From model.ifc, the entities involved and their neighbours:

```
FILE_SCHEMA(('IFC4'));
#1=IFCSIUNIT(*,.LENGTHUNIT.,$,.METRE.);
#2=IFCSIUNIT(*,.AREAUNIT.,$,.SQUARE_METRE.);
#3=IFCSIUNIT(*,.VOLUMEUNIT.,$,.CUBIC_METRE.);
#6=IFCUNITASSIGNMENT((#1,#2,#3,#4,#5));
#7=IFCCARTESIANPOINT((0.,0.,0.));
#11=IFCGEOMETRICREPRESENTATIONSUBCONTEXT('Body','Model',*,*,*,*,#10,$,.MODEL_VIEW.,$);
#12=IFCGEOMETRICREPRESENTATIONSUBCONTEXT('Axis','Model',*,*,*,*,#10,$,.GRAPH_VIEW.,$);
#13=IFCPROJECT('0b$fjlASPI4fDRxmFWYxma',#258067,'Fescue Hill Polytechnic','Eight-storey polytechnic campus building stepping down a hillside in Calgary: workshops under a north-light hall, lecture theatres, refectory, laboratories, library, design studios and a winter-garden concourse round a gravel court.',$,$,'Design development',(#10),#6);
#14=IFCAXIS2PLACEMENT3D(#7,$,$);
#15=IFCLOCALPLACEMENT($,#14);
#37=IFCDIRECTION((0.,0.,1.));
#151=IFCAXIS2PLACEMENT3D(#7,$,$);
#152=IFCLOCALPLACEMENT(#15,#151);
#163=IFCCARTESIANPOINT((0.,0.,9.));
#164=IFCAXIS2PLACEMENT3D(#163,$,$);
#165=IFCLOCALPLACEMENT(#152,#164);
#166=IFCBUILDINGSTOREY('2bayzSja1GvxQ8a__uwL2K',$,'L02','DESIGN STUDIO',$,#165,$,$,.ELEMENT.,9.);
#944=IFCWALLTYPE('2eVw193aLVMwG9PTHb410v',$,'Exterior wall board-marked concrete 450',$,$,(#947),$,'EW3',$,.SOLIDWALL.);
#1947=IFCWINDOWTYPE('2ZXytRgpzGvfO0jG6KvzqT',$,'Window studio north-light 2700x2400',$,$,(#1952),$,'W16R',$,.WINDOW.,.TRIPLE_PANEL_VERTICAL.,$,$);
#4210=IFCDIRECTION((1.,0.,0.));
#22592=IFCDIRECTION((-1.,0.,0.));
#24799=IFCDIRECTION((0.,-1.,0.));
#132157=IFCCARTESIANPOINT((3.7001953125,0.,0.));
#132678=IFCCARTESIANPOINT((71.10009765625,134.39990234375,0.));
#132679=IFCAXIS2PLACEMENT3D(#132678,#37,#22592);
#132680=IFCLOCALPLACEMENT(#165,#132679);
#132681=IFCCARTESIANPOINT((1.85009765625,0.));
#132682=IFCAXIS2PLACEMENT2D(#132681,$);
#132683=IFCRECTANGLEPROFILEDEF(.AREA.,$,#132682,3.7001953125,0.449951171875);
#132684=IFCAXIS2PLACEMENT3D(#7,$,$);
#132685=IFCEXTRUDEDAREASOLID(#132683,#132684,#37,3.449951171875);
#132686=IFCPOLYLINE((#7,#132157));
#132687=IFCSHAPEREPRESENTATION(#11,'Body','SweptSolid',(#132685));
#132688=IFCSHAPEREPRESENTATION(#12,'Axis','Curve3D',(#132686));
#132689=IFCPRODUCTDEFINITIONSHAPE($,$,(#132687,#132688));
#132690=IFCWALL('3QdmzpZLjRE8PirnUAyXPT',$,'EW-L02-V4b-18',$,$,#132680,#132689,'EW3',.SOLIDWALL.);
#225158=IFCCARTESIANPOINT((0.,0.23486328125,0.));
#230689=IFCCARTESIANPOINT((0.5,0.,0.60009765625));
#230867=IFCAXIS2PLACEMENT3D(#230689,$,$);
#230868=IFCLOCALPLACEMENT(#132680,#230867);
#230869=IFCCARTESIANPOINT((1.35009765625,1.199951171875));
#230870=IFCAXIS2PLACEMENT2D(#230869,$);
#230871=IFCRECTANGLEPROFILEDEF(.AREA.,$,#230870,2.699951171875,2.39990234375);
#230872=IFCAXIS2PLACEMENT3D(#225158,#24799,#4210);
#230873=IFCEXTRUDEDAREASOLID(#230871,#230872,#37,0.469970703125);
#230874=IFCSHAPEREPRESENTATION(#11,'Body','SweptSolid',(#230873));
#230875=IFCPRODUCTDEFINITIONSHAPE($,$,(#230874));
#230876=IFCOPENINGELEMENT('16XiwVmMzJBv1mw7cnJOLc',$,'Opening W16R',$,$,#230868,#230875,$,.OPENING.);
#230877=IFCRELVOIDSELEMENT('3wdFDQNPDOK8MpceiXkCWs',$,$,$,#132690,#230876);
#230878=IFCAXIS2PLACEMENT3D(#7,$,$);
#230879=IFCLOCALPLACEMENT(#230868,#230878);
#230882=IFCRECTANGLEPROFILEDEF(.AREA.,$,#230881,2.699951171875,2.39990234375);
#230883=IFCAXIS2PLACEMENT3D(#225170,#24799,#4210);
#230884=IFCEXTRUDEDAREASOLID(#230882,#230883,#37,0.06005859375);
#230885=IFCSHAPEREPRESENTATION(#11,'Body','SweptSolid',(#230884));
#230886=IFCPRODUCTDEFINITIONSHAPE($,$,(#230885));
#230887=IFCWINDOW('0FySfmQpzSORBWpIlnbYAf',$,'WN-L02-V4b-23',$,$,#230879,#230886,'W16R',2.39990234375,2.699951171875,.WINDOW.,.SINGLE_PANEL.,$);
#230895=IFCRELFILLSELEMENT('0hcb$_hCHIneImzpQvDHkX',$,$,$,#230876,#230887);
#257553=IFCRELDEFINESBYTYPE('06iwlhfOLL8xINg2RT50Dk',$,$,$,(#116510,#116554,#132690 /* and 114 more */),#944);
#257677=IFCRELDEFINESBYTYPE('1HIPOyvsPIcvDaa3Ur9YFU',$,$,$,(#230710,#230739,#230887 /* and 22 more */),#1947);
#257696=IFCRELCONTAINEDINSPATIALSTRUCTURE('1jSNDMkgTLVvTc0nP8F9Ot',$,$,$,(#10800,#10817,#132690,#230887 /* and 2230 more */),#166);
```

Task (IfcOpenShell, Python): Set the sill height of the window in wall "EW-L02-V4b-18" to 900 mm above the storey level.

```python
import numpy as np
import ifcopenshell
import ifcopenshell.api.geometry
import ifcopenshell.geom
import ifcopenshell.util.element
import ifcopenshell.util.placement
import ifcopenshell.util.shape
import ifcopenshell.util.unit

model = ifcopenshell.open("model.ifc")
unit_scale = ifcopenshell.util.unit.calculate_unit_scale(model)

window = model.by_guid("0FySfmQpzSORBWpIlnbYAf")
opening = window.FillsVoids[0].RelatingOpeningElement
storey = ifcopenshell.util.element.get_container(window, ifc_class="IfcBuildingStorey")
level = ifcopenshell.util.placement.get_local_placement(storey.ObjectPlacement)[2, 3]

# The opening's origin need not be at the sill, so measure its lowest point.
shape = ifcopenshell.geom.create_shape(ifcopenshell.geom.settings(), opening)
bottom = ifcopenshell.util.shape.get_shape_bottom_elevation(shape, shape.geometry) / unit_scale
dz = level + 0.9 - bottom

shift = np.array([0.0, 0.0, dz])
# The window is placed relative to its opening, so it follows when the opening moves.
matrix = ifcopenshell.util.placement.get_local_placement(opening.ObjectPlacement)
matrix[:3, 3] += shift
ifcopenshell.api.geometry.edit_object_placement(
    model, product=opening, matrix=matrix, is_si=False, should_transform_children=True
)

print(f"moved by {dz * unit_scale:+.3f} m")

model.write("model_updated.ifc")
```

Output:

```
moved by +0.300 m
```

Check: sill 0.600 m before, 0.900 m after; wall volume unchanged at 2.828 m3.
